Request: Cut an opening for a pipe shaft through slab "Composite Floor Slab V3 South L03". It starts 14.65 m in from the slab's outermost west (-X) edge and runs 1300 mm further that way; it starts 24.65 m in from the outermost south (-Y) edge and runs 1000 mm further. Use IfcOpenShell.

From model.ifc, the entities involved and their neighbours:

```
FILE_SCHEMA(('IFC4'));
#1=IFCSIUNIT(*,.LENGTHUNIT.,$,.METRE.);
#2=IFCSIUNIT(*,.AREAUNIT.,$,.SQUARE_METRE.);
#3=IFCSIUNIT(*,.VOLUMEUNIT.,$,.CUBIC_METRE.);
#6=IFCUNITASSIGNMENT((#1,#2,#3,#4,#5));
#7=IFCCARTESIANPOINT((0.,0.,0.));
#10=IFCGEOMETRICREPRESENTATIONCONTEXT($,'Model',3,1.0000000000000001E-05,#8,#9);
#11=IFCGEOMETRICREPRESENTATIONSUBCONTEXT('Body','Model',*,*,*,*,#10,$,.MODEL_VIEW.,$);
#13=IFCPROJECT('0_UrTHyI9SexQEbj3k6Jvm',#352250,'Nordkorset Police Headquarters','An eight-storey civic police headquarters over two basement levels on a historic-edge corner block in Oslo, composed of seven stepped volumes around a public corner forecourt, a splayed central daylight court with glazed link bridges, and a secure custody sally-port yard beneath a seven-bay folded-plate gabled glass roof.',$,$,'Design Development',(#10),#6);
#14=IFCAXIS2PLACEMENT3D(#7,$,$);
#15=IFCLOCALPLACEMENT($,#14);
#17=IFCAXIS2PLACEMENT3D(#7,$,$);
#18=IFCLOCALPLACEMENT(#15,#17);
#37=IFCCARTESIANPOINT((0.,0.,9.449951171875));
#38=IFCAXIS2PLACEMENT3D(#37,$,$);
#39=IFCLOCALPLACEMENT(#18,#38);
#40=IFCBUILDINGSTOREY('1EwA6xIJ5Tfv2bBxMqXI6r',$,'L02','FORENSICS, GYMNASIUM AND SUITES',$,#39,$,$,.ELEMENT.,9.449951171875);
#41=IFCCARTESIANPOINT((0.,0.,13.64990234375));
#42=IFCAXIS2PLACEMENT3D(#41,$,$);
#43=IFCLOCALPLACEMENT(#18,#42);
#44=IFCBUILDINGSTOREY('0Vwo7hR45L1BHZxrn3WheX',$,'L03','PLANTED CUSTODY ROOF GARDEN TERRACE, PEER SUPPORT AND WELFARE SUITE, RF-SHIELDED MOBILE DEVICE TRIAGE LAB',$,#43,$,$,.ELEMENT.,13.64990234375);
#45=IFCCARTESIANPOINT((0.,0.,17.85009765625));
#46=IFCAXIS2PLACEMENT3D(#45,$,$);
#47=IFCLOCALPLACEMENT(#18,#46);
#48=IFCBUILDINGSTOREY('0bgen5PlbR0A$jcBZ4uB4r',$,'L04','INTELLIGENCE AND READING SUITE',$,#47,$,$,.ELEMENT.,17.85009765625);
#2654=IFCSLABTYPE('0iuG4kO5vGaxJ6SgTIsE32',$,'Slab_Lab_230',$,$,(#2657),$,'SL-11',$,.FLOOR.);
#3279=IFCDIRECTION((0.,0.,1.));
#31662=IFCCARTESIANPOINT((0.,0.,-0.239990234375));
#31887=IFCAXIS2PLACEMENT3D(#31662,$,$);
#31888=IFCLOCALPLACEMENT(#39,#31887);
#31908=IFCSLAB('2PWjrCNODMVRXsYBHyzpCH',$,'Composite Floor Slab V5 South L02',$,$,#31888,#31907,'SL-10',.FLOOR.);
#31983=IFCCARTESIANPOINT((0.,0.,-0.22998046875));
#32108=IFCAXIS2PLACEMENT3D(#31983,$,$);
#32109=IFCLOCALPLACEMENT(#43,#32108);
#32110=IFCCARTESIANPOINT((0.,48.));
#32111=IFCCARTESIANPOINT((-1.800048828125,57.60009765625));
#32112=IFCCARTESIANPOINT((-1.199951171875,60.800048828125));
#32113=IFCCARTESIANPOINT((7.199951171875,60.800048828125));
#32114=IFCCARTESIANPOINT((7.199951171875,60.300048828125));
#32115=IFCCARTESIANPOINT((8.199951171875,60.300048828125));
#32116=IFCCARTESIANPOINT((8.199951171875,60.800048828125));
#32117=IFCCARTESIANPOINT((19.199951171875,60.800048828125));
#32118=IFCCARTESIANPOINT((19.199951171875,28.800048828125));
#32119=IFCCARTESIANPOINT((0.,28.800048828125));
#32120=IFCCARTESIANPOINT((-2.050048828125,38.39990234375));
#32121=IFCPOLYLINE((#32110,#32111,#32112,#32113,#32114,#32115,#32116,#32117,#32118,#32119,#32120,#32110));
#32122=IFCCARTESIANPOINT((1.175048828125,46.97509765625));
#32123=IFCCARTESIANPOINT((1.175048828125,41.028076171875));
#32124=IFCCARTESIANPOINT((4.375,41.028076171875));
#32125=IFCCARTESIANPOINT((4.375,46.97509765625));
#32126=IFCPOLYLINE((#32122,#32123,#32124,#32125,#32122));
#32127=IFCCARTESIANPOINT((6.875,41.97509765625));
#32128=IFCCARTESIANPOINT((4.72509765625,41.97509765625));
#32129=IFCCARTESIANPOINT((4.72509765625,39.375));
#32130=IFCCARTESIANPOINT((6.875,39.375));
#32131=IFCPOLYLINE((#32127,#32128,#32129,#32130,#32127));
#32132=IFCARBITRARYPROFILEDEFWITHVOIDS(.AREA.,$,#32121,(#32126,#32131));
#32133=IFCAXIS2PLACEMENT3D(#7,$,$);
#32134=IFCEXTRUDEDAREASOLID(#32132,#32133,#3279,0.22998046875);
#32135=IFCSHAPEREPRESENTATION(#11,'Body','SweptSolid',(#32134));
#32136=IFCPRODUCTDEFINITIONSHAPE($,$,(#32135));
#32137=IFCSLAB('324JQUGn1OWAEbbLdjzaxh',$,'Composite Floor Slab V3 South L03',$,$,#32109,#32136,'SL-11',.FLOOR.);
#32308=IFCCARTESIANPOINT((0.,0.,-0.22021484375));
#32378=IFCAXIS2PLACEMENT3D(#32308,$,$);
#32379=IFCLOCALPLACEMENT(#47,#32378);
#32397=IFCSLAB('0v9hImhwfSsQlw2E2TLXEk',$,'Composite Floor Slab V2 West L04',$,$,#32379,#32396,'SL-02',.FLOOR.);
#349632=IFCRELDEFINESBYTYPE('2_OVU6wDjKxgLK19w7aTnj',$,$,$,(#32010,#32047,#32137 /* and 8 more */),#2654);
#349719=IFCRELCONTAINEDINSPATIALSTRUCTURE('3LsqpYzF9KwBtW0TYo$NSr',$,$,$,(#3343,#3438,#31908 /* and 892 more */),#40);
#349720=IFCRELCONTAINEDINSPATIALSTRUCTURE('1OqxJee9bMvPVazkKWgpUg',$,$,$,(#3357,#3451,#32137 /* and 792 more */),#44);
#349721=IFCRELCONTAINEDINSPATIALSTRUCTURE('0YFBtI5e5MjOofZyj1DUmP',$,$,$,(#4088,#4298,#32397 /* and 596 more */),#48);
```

```python
import numpy as np
import ifcopenshell
import ifcopenshell.api.feature
import ifcopenshell.api.geometry
import ifcopenshell.api.root
import ifcopenshell.geom
import ifcopenshell.util.placement
import ifcopenshell.util.representation
import ifcopenshell.util.shape
import ifcopenshell.util.unit

model = ifcopenshell.open("model.ifc")
unit_scale = ifcopenshell.util.unit.calculate_unit_scale(model)
settings = ifcopenshell.geom.settings()


def volume(element):
    """Net volume in cubic metres, openings subtracted."""
    shape = ifcopenshell.geom.create_shape(settings, element)
    return ifcopenshell.util.shape.get_volume(shape.geometry)


slab = model.by_guid("324JQUGn1OWAEbbLdjzaxh")
before = volume(slab)

# Extent in the slab's own axes, in metres. The edges named are its -X and -Y sides.
slab_shape = ifcopenshell.geom.create_shape(settings, slab)
vertices = ifcopenshell.util.shape.get_vertices(slab_shape.geometry)
x_min, y_min, bottom = vertices.min(axis=0)
top = vertices[:, 2].max()

opening = ifcopenshell.api.root.create_entity(model, ifc_class="IfcOpeningElement", name="Pipe shaft opening", predefined_type="OPENING")
context = ifcopenshell.util.representation.get_context(model, "Model", "Body", "MODEL_VIEW")
width, depth = 1.3, 1
outline = [(0.0, 0.0), (width, 0.0), (width, depth), (0.0, depth), (0.0, 0.0)]
# Overshoot both faces by 50 mm so the cut is clean.
shape = ifcopenshell.api.geometry.add_slab_representation(
    model, context=context, depth=top - bottom + 0.1, polyline=outline
)
ifcopenshell.api.geometry.assign_representation(model, product=opening, representation=shape)

matrix = ifcopenshell.util.placement.get_local_placement(slab.ObjectPlacement)
matrix[:, 3] = matrix @ np.append(np.array([x_min + 14.65, y_min + 24.65, bottom - 0.05]) / unit_scale, 1.0)
ifcopenshell.api.geometry.edit_object_placement(model, product=opening, matrix=matrix, is_si=False)
ifcopenshell.api.feature.add_feature(model, feature=opening, element=slab)

after = volume(slab)

print(f"slab volume {before:.3f} -> {after:.3f} m3")

model.write("model_rev.ifc")
```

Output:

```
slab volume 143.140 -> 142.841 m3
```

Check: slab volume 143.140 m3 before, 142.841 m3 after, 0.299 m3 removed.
